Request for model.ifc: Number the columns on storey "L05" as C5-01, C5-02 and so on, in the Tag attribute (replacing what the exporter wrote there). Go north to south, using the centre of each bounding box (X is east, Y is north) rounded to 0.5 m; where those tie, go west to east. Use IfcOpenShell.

First a look at what the model holds.

```python
import ifcopenshell
import ifcopenshell.util.element
import ifcopenshell.util.placement

model = ifcopenshell.open("model.ifc")
print(model.schema)
storey = next(s for s in model.by_type("IfcBuildingStorey") if s.Name == "L05")
columns = [e for e in ifcopenshell.util.element.get_decomposition(storey) if e.is_a("IfcColumn")]
for e in sorted(columns, key=lambda e: e.id()):
    origin = ifcopenshell.util.placement.get_local_placement(e.ObjectPlacement)[:3, 3]
    print(e.id(), e.Tag, e.Name, origin.round(2) + 0.0, sep=" | ")
```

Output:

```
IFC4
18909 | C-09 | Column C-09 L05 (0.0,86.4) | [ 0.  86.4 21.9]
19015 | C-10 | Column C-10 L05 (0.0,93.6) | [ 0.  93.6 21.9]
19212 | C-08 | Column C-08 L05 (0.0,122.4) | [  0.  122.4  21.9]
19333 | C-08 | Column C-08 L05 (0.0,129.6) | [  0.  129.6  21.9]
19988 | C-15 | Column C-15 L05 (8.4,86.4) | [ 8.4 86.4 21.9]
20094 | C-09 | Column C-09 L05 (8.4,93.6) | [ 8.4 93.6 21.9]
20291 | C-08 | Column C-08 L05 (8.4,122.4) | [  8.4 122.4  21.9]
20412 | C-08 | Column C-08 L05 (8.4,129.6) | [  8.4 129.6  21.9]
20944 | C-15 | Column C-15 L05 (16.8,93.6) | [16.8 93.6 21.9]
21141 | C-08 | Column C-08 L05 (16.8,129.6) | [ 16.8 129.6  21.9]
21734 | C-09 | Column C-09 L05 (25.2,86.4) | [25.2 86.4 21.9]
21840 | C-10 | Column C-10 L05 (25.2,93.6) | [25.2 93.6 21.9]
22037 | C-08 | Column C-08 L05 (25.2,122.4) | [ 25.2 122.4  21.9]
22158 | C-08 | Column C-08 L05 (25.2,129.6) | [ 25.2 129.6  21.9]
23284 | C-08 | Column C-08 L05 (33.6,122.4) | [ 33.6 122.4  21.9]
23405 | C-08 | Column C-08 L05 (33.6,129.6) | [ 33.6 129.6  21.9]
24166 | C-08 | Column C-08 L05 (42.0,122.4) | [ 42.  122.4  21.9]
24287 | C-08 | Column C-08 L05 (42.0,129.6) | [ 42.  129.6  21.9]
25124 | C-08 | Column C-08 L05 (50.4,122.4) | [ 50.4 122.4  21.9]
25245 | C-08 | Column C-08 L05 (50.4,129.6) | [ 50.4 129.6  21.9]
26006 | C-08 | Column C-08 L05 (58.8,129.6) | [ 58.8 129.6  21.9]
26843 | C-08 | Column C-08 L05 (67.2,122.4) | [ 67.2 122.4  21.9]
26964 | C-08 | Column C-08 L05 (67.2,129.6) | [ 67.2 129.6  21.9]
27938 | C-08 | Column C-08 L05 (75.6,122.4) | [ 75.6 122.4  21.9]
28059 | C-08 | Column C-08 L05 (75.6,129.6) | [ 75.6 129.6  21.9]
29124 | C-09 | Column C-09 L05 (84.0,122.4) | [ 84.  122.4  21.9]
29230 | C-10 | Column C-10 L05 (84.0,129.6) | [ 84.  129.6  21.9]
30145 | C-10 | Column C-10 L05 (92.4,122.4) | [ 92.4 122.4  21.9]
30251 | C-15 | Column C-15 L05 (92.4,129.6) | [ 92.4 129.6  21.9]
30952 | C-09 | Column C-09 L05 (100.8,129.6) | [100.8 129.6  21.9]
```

```python
import ifcopenshell
import ifcopenshell.geom
import ifcopenshell.util.element
import ifcopenshell.util.shape

model = ifcopenshell.open("model.ifc")
settings = ifcopenshell.geom.settings()
settings.set("use-world-coords", True)


def centre(element):
    shape = ifcopenshell.geom.create_shape(settings, element)
    return ifcopenshell.util.shape.get_bbox_centroid(shape.geometry)


storey = next(s for s in model.by_type("IfcBuildingStorey") if s.Name == "L05")
columns = [e for e in ifcopenshell.util.element.get_decomposition(storey) if e.is_a("IfcColumn")]

# Insertion points can sit at a corner or the storey origin, so sort by the geometry (in metres).
centres = {e: centre(e) for e in columns}
columns.sort(key=lambda e: (-round(centres[e][1] / 0.5), centres[e][0]))

for i, e in enumerate(columns, start=1):
    number = f"C5-{i:02d}"
    e.Tag = number
    print(e.id(), number)

model.write("model-out.ifc")
```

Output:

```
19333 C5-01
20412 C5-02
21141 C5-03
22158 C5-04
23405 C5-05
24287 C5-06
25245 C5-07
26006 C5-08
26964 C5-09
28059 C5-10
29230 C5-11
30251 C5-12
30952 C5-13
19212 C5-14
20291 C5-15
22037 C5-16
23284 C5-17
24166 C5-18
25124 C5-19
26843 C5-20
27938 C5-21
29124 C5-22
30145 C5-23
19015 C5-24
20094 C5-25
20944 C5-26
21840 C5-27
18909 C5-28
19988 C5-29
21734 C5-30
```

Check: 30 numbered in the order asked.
